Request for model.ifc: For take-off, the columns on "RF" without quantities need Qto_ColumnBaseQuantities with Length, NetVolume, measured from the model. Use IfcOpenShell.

First a look at what the model holds.

```python
import ifcopenshell
import ifcopenshell.util.element
import ifcopenshell.util.unit

model = ifcopenshell.open("model.ifc")
print(model.schema)
for unit_type in ("LENGTHUNIT", "AREAUNIT", "VOLUMEUNIT"):
    print(unit_type, ifcopenshell.util.unit.calculate_unit_scale(model, unit_type))
storey = next(s for s in model.by_type("IfcBuildingStorey") if s.Name == "RF")
columns = [e for e in ifcopenshell.util.element.get_decomposition(storey) if e.is_a("IfcColumn")]
for e in sorted(columns, key=lambda e: e.id()):
    print(e.id(), e.is_a(), e.Name, list(ifcopenshell.util.element.get_psets(e, qtos_only=True)), sep=" | ")
```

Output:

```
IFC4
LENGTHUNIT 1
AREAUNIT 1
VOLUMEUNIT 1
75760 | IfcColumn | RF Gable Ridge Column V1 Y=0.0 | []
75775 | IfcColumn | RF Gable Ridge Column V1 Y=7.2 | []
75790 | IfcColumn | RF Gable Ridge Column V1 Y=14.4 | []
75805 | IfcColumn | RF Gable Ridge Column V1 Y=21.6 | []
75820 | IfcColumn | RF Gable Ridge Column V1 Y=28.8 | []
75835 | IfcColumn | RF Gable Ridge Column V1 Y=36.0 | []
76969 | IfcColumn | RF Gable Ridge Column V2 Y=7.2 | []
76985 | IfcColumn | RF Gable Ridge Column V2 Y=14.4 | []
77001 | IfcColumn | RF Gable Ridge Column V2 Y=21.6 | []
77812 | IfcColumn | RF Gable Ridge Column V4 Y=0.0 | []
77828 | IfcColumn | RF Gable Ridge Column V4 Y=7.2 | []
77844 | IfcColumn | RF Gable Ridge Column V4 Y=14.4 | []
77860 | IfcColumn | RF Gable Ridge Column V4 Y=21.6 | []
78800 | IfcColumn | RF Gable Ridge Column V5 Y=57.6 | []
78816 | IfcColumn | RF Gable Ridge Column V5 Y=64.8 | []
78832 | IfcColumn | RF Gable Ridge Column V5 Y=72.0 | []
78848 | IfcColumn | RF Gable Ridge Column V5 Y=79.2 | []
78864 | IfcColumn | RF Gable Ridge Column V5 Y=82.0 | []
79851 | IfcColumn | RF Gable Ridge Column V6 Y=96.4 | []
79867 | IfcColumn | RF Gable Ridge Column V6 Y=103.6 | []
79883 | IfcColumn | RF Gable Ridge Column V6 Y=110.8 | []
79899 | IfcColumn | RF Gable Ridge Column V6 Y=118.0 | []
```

```python
import ifcopenshell
import ifcopenshell.api.pset
import ifcopenshell.geom
import ifcopenshell.util.element
import ifcopenshell.util.shape
import ifcopenshell.util.unit

model = ifcopenshell.open("model.ifc")
unit_scale = ifcopenshell.util.unit.calculate_unit_scale(model)
volume_scale = ifcopenshell.util.unit.calculate_unit_scale(model, "VOLUMEUNIT")
settings = ifcopenshell.geom.settings()

storey = next(s for s in model.by_type("IfcBuildingStorey") if s.Name == "RF")
columns = [e for e in ifcopenshell.util.element.get_decomposition(storey) if e.is_a("IfcColumn")]

for e in sorted(columns, key=lambda e: e.id()):
    if ifcopenshell.util.element.get_psets(e, qtos_only=True, should_inherit=False):
        continue
    # Geometry comes back in metres, in the element's own axes.
    shape = ifcopenshell.geom.create_shape(settings, e)
    values = {
        "Length": ifcopenshell.util.shape.get_z(shape.geometry) / unit_scale,
        "NetVolume": ifcopenshell.util.shape.get_volume(shape.geometry) / volume_scale,
    }
    qto = ifcopenshell.api.pset.add_qto(model, product=e, name="Qto_ColumnBaseQuantities")
    ifcopenshell.api.pset.edit_qto(model, qto=qto, properties=values)
    print(e.id(), {k: round(v, 3) for k, v in values.items()})

model.write("model_v2.ifc")
```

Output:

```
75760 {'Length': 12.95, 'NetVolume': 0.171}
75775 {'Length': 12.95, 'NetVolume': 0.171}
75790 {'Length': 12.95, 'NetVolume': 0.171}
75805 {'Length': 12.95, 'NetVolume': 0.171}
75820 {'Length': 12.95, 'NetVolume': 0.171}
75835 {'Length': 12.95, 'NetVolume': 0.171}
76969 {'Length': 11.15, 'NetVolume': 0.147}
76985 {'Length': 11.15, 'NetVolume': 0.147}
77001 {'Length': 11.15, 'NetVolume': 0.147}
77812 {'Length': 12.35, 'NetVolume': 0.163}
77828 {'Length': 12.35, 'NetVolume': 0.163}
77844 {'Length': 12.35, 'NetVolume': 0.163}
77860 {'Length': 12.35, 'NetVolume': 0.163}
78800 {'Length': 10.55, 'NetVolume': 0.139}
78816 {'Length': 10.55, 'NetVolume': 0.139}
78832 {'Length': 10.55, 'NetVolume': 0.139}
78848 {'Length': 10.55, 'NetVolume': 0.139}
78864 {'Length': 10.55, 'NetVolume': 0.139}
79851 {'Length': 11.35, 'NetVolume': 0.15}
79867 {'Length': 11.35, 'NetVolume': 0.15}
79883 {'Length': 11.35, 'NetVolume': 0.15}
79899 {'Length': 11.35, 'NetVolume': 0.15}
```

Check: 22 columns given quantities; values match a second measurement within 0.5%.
